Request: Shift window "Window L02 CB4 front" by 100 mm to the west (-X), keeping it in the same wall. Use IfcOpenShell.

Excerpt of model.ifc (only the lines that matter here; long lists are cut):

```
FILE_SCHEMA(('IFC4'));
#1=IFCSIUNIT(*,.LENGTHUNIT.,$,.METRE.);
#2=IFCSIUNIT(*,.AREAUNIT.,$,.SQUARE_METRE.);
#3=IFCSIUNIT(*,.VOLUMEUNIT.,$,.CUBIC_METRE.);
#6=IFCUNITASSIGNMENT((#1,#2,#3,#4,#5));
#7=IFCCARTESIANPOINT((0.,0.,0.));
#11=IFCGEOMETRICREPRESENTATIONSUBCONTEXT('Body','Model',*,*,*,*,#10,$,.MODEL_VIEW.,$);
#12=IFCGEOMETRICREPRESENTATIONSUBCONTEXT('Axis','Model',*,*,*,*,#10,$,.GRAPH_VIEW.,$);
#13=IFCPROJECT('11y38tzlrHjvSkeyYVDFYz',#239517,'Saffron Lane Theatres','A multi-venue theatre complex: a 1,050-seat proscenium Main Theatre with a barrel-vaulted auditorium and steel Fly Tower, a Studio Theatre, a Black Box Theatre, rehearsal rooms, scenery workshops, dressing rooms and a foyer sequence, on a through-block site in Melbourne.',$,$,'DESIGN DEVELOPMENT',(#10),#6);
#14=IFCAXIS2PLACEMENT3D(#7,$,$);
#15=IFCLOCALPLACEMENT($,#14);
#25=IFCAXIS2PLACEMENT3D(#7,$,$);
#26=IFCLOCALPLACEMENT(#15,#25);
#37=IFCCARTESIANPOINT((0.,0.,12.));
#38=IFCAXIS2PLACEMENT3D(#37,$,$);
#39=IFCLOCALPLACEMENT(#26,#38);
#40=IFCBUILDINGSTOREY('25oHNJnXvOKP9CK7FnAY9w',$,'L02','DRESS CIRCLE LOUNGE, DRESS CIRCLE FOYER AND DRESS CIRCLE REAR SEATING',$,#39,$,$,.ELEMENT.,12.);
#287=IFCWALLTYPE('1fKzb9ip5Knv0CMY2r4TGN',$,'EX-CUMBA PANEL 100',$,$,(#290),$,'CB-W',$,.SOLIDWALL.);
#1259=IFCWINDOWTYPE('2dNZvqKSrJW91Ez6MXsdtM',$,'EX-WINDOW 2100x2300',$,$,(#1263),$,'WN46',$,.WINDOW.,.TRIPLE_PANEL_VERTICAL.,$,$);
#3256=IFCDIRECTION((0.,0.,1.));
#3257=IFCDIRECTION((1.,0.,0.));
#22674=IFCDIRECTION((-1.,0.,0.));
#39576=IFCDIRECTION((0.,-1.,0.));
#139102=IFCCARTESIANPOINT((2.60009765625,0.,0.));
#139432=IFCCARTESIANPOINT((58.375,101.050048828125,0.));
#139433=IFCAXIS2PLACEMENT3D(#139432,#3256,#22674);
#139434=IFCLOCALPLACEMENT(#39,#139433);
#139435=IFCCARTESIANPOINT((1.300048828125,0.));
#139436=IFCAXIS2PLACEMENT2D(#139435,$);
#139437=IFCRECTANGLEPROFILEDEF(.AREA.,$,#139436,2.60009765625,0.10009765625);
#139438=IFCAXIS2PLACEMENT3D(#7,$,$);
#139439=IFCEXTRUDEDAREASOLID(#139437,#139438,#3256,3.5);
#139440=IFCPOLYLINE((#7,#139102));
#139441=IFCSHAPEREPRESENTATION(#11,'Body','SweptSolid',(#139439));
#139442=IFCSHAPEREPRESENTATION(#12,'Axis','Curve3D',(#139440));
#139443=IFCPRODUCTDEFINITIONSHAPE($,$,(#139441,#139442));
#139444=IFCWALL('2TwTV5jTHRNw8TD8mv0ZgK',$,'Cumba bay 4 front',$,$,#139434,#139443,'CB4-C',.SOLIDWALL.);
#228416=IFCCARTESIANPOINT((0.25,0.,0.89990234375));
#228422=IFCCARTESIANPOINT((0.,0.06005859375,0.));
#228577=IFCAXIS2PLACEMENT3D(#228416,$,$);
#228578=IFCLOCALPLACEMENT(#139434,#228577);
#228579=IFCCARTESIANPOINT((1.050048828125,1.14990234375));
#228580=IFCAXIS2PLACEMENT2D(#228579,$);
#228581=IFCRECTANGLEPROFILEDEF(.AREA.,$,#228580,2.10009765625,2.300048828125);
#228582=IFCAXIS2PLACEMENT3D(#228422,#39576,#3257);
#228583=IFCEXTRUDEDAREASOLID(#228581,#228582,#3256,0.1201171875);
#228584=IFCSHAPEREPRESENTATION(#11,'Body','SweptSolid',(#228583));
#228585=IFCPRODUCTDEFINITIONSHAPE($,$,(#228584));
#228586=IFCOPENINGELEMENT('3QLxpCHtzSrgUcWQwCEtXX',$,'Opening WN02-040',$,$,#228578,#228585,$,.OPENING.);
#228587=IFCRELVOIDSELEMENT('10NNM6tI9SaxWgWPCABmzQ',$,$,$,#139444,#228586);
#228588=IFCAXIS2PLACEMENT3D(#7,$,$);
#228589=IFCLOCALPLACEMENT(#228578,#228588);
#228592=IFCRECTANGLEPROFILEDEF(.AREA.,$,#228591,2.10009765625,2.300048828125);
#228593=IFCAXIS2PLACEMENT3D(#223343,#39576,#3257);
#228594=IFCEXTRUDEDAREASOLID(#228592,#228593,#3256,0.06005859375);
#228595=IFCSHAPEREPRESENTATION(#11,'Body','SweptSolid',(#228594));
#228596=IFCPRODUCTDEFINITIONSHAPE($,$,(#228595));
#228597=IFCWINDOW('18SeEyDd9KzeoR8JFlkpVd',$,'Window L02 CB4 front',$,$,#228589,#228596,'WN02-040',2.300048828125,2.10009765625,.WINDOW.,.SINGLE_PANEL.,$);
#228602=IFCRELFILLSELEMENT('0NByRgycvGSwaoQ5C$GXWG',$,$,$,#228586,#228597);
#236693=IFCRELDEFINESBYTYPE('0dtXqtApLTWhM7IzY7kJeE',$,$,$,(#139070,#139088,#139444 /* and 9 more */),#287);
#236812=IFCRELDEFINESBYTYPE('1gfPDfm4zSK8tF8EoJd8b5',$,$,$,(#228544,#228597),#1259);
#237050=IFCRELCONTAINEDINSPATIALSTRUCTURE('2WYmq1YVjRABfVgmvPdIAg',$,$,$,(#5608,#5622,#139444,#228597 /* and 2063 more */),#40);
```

```python
import ifcopenshell
import ifcopenshell.api.geometry
import ifcopenshell.util.placement

model = ifcopenshell.open("model.ifc")

window = model.by_guid("18SeEyDd9KzeoR8JFlkpVd")
opening = window.FillsVoids[0].RelatingOpeningElement
wall = opening.VoidsElements[0].RelatingBuildingElement

wall_matrix = ifcopenshell.util.placement.get_local_placement(wall.ObjectPlacement)
shift = wall_matrix[:3, 0] * 0.1
before = ifcopenshell.util.placement.get_local_placement(window.ObjectPlacement)[:3, 3].copy()

# The window is placed relative to its opening, so it follows when the opening moves.
matrix = ifcopenshell.util.placement.get_local_placement(opening.ObjectPlacement)
matrix[:3, 3] += shift
ifcopenshell.api.geometry.edit_object_placement(
    model, product=opening, matrix=matrix, is_si=False, should_transform_children=True
)

after = ifcopenshell.util.placement.get_local_placement(window.ObjectPlacement)[:3, 3]
print("window moved by", (after - before).round(3) + 0.0)

model.write("model_updated.ifc")
```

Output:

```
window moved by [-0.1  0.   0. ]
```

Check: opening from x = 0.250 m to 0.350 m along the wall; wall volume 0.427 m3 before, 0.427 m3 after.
